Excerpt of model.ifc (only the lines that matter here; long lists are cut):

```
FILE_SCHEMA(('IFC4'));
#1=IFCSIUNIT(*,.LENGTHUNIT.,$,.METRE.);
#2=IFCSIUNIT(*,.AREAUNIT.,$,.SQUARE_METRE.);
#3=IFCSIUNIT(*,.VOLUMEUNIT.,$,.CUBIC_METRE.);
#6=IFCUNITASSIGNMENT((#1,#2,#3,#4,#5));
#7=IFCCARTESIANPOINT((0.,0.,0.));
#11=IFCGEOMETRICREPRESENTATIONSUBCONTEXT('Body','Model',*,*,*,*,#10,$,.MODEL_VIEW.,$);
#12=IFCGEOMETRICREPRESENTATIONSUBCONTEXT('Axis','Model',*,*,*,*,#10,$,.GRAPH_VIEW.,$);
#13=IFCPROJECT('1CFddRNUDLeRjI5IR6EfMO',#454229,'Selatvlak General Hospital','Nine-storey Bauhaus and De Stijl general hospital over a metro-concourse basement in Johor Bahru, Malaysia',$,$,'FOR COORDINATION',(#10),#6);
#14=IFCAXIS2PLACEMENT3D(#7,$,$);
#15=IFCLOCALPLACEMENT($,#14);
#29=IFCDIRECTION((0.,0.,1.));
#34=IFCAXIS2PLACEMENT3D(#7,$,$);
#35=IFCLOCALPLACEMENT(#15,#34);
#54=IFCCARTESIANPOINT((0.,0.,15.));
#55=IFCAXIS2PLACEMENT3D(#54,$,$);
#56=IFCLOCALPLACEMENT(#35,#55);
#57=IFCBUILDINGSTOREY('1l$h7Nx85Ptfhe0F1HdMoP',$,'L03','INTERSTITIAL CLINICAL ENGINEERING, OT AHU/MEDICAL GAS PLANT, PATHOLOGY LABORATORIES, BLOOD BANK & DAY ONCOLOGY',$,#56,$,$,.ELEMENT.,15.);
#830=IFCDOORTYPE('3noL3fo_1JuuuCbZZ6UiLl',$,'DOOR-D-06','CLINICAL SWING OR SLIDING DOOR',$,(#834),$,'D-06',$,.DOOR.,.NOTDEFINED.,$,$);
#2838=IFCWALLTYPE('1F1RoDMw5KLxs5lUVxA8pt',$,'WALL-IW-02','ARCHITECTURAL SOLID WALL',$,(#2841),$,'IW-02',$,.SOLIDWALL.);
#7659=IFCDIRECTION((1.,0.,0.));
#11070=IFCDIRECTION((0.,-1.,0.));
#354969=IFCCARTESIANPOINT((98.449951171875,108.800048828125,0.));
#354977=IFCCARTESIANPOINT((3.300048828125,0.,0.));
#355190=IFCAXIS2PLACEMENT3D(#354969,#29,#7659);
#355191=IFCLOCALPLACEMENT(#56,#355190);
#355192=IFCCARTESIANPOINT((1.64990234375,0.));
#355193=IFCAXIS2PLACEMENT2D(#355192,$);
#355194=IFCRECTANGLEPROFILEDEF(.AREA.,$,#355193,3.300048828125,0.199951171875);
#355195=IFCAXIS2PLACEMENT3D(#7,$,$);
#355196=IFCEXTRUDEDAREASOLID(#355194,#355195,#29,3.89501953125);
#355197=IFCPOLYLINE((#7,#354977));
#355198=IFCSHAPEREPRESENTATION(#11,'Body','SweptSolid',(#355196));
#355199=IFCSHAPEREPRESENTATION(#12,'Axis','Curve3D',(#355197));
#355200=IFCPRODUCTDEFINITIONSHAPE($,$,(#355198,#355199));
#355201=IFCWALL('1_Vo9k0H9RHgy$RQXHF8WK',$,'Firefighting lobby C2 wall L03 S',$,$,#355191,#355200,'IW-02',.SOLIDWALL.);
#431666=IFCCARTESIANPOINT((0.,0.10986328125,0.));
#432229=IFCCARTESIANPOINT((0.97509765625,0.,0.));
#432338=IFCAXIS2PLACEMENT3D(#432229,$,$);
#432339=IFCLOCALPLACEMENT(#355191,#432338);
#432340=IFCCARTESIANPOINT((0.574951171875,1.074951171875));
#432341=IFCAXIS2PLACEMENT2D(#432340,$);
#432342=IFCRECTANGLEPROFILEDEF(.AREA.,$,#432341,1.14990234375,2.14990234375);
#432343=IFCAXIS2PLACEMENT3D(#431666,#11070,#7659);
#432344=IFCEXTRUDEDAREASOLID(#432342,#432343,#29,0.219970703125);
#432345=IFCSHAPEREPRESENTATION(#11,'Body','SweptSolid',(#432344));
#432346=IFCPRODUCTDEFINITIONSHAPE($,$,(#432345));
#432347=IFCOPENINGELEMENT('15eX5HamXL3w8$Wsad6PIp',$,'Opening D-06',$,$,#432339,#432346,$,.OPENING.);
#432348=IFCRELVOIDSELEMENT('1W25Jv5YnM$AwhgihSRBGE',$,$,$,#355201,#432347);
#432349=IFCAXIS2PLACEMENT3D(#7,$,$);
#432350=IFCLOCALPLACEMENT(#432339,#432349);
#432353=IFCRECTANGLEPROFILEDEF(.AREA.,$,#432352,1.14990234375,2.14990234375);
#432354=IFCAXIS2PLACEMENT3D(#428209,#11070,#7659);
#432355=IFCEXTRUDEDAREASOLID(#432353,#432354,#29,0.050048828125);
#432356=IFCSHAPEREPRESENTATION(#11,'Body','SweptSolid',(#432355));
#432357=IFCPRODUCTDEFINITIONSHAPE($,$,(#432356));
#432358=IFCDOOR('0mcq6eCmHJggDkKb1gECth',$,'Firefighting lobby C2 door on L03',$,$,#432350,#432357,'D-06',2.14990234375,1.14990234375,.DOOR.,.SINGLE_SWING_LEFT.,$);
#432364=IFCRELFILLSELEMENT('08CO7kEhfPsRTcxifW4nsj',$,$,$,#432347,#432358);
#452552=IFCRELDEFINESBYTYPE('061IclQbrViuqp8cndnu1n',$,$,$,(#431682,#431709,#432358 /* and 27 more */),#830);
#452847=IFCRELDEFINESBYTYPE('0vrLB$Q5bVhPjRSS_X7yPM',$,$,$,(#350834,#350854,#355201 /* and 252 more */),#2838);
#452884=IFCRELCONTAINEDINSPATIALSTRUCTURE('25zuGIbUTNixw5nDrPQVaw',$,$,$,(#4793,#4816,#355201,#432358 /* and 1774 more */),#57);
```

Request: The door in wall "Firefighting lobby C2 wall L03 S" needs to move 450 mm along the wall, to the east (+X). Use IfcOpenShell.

```python
import ifcopenshell
import ifcopenshell.api.geometry
import ifcopenshell.util.placement

model = ifcopenshell.open("model.ifc")

door = model.by_guid("0mcq6eCmHJggDkKb1gECth")
opening = door.FillsVoids[0].RelatingOpeningElement
wall = opening.VoidsElements[0].RelatingBuildingElement

wall_matrix = ifcopenshell.util.placement.get_local_placement(wall.ObjectPlacement)
shift = wall_matrix[:3, 0] * 0.45
before = ifcopenshell.util.placement.get_local_placement(door.ObjectPlacement)[:3, 3].copy()

# The door is placed relative to its opening, so it follows when the opening moves.
matrix = ifcopenshell.util.placement.get_local_placement(opening.ObjectPlacement)
matrix[:3, 3] += shift
ifcopenshell.api.geometry.edit_object_placement(
    model, product=opening, matrix=matrix, is_si=False, should_transform_children=True
)

after = ifcopenshell.util.placement.get_local_placement(door.ObjectPlacement)[:3, 3]
print("door moved by", (after - before).round(3) + 0.0)

model.write("model_v2.ifc")
```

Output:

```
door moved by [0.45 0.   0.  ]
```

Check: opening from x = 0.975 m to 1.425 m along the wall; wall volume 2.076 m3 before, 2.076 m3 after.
